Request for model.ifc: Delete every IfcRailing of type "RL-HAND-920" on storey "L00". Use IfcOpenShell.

First a look at what the model holds.

```python
import ifcopenshell
import ifcopenshell.util.element

model = ifcopenshell.open("model.ifc")
print(model.schema)
storey = next(s for s in model.by_type("IfcBuildingStorey") if s.Name == "L00")
railings = [e for e in ifcopenshell.util.element.get_decomposition(storey) if e.is_a("IfcRailing")]
seen = {}
for e in railings:
    element_type = ifcopenshell.util.element.get_type(e)
    name = element_type.Name if element_type not in (None, e) else None
    seen[name] = seen.get(name, 0) + 1
for name, count in sorted(seen.items(), key=str):
    print(count, "x", name)
```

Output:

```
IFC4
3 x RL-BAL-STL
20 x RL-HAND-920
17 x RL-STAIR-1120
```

```python
import ifcopenshell
import ifcopenshell.api.root
import ifcopenshell.util.element

model = ifcopenshell.open("model.ifc")

storey = next(s for s in model.by_type("IfcBuildingStorey") if s.Name == "L00")
railings = [e for e in ifcopenshell.util.element.get_decomposition(storey) if e.is_a("IfcRailing")]
targets = [e for e in railings if (t := ifcopenshell.util.element.get_type(e)) not in (None, e) and t.Name == "RL-HAND-920"]

for e in targets:
    ifcopenshell.api.root.remove_product(model, product=e)
print(len(targets), "removed")

model.write("model_rev.ifc")
```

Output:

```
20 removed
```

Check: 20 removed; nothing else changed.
